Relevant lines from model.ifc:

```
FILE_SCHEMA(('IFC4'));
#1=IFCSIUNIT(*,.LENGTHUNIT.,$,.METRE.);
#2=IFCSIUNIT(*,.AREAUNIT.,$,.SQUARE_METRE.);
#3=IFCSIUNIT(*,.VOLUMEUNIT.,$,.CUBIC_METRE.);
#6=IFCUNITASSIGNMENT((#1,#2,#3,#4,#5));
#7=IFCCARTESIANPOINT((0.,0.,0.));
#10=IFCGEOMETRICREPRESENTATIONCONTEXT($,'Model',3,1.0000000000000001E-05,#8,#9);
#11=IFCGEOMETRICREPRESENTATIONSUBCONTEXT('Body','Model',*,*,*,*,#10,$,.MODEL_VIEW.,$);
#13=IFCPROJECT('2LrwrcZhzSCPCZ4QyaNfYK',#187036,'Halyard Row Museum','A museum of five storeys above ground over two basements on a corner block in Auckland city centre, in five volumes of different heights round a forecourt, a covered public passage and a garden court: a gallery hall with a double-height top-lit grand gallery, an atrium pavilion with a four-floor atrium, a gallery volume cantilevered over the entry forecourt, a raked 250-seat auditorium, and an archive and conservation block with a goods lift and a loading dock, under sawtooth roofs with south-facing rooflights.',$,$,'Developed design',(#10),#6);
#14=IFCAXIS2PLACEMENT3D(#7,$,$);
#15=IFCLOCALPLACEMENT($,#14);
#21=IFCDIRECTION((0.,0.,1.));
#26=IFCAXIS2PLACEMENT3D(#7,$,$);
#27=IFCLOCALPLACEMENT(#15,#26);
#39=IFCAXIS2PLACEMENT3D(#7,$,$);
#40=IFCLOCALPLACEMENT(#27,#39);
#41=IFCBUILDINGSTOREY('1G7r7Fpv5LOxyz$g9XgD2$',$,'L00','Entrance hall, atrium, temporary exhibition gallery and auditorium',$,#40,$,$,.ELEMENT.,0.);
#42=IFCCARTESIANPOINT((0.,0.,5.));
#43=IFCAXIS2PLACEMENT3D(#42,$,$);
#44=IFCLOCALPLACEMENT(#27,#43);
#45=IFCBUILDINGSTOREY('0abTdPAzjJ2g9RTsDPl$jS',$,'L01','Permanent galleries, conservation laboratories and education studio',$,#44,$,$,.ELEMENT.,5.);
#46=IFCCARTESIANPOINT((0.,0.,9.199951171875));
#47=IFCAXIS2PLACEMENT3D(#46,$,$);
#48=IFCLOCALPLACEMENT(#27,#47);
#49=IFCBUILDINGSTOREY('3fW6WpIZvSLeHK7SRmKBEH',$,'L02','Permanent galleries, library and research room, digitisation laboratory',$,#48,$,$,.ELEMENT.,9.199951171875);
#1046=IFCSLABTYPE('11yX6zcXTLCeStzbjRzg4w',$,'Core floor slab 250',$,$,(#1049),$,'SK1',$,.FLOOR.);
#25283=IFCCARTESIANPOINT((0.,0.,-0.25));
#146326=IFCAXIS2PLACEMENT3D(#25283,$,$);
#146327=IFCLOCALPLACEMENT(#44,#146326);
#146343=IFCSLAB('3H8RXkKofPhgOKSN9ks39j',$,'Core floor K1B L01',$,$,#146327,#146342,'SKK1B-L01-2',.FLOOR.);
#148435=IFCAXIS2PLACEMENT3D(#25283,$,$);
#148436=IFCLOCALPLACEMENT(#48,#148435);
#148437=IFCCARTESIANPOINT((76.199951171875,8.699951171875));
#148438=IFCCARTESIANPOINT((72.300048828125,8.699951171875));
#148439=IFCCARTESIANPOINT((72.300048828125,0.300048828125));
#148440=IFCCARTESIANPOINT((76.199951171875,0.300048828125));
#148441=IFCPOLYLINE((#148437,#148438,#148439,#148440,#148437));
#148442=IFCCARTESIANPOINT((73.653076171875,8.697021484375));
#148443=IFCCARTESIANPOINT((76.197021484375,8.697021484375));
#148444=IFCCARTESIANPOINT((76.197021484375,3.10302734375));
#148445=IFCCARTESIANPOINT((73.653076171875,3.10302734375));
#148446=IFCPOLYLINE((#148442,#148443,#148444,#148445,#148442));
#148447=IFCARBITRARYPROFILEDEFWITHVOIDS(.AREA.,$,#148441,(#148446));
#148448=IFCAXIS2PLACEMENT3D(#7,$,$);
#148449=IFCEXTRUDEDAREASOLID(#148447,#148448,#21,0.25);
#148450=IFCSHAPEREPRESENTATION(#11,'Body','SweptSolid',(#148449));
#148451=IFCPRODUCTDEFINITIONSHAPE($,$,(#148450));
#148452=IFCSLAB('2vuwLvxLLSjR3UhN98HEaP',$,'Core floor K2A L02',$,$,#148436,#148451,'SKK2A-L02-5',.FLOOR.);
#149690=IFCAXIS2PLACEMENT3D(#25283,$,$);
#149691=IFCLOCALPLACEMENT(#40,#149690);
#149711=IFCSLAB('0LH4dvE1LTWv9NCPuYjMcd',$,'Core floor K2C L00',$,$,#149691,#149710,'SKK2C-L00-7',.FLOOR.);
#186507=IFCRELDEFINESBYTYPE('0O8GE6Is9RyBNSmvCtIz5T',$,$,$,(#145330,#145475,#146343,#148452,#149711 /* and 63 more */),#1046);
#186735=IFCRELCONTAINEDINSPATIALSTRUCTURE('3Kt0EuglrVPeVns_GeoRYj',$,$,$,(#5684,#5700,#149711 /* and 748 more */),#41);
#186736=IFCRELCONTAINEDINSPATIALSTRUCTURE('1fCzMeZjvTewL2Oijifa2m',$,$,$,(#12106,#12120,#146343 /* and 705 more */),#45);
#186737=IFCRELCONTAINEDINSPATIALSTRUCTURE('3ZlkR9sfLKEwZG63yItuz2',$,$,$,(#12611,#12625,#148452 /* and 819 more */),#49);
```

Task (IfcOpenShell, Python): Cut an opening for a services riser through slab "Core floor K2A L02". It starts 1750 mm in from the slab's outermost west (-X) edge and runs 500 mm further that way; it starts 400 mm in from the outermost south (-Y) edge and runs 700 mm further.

```python
import numpy as np
import ifcopenshell
import ifcopenshell.api.feature
import ifcopenshell.api.geometry
import ifcopenshell.api.root
import ifcopenshell.geom
import ifcopenshell.util.placement
import ifcopenshell.util.representation
import ifcopenshell.util.shape
import ifcopenshell.util.unit

model = ifcopenshell.open("model.ifc")
unit_scale = ifcopenshell.util.unit.calculate_unit_scale(model)
settings = ifcopenshell.geom.settings()


def volume(element):
    """Net volume in cubic metres, openings subtracted."""
    shape = ifcopenshell.geom.create_shape(settings, element)
    return ifcopenshell.util.shape.get_volume(shape.geometry)


slab = model.by_id(148452)
before = volume(slab)

# Extent in the slab's own axes, in metres. The edges named are its -X and -Y sides.
slab_shape = ifcopenshell.geom.create_shape(settings, slab)
vertices = ifcopenshell.util.shape.get_vertices(slab_shape.geometry)
x_min, y_min, bottom = vertices.min(axis=0)
top = vertices[:, 2].max()

opening = ifcopenshell.api.root.create_entity(model, ifc_class="IfcOpeningElement", name="Services riser opening", predefined_type="OPENING")
context = ifcopenshell.util.representation.get_context(model, "Model", "Body", "MODEL_VIEW")
width, depth = 0.5, 0.7
outline = [(0.0, 0.0), (width, 0.0), (width, depth), (0.0, depth), (0.0, 0.0)]
# Overshoot both faces by 50 mm so the cut is clean.
shape = ifcopenshell.api.geometry.add_slab_representation(
    model, context=context, depth=top - bottom + 0.1, polyline=outline
)
ifcopenshell.api.geometry.assign_representation(model, product=opening, representation=shape)

matrix = ifcopenshell.util.placement.get_local_placement(slab.ObjectPlacement)
matrix[:, 3] = matrix @ np.append(np.array([x_min + 1.75, y_min + 0.4, bottom - 0.05]) / unit_scale, 1.0)
ifcopenshell.api.geometry.edit_object_placement(model, product=opening, matrix=matrix, is_si=False)
ifcopenshell.api.feature.add_feature(model, feature=opening, element=slab)

after = volume(slab)

print(f"slab volume {before:.3f} -> {after:.3f} m3")

model.write("model-out.ifc")
```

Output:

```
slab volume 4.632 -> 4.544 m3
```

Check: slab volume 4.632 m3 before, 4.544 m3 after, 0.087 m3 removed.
